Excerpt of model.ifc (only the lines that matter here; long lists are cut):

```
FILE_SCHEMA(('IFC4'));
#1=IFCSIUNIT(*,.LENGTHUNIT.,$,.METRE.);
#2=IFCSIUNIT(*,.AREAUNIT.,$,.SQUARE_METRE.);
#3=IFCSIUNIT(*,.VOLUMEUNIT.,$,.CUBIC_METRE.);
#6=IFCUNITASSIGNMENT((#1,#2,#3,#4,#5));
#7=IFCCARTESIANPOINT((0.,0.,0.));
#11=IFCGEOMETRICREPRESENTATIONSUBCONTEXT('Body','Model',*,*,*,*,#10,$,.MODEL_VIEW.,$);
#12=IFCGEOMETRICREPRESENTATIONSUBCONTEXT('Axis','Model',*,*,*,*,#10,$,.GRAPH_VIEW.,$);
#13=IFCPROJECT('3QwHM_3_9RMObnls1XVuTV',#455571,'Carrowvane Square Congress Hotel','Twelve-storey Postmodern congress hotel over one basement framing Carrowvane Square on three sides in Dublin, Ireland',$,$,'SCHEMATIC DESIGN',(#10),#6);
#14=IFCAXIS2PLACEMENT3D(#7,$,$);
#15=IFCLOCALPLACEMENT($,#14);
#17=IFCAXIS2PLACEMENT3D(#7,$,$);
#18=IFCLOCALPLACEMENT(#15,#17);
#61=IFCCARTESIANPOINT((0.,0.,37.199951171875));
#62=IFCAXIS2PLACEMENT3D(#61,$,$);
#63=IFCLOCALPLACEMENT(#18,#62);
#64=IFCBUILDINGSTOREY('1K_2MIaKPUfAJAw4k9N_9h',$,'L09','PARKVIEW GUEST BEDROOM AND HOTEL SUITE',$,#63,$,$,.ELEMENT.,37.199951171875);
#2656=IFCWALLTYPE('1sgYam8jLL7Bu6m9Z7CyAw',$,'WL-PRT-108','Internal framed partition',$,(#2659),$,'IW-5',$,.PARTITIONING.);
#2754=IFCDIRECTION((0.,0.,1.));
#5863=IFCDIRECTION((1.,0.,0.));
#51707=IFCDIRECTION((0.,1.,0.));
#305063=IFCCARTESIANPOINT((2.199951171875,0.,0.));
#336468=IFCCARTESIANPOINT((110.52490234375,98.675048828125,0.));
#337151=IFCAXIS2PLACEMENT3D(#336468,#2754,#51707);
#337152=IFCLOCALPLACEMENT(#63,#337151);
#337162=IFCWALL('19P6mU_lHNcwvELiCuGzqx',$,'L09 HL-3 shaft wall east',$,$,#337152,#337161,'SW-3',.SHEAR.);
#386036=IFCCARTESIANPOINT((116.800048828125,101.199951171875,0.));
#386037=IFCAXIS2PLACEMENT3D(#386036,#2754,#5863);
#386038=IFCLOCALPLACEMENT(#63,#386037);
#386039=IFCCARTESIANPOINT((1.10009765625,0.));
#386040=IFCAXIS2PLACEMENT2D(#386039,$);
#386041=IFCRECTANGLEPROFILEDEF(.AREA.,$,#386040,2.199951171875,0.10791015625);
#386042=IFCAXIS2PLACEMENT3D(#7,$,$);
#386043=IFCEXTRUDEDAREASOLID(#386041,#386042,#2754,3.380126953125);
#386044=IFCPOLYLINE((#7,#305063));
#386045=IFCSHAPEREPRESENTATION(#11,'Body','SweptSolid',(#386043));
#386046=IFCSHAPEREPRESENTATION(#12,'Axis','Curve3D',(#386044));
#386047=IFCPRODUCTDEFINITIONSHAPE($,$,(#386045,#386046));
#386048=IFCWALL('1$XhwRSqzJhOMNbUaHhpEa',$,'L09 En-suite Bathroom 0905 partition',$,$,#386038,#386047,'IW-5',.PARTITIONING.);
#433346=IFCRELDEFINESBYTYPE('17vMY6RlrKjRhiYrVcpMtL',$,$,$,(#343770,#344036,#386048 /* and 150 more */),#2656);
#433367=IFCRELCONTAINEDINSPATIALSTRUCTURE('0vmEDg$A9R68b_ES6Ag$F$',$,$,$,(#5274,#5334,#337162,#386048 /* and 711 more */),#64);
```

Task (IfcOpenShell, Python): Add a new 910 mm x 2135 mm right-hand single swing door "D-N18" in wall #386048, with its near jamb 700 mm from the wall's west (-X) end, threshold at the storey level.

```python
import numpy as np
import ifcopenshell
import ifcopenshell.api.feature
import ifcopenshell.api.geometry
import ifcopenshell.api.root
import ifcopenshell.api.spatial
import ifcopenshell.geom
import ifcopenshell.util.element
import ifcopenshell.util.placement
import ifcopenshell.util.representation
import ifcopenshell.util.shape
import ifcopenshell.util.unit

model = ifcopenshell.open("model.ifc")
unit_scale = ifcopenshell.util.unit.calculate_unit_scale(model)
settings = ifcopenshell.geom.settings()


def volume(element):
    """Net volume in cubic metres, openings subtracted."""
    shape = ifcopenshell.geom.create_shape(settings, element)
    return ifcopenshell.util.shape.get_volume(shape.geometry)


wall = model.by_guid("1$XhwRSqzJhOMNbUaHhpEa")
storey = ifcopenshell.util.element.get_container(wall, ifc_class="IfcBuildingStorey")
context = ifcopenshell.util.representation.get_context(model, "Model", "Body", "MODEL_VIEW")
before = volume(wall)

width, height, from_end, sill = 0.91, 2.135, 0.7, 0.0  # metres

# The wall runs along its own X axis, and the end named is its -X end.
wall_shape = ifcopenshell.geom.create_shape(settings, wall)
x, y, z = ifcopenshell.util.shape.get_vertices(wall_shape.geometry).T
start = x.min() + from_end
face, thickness = float(y.min()), float(y.max() - y.min())
wall_matrix = ifcopenshell.util.placement.get_local_placement(wall.ObjectPlacement)
level = ifcopenshell.util.placement.get_local_placement(storey.ObjectPlacement)[2, 3]


def in_wall(x, y):
    """Placement at x, y metres in the wall's axes, at sill height."""
    matrix = wall_matrix.copy()
    matrix[:, 3] = wall_matrix @ np.array([x / unit_scale, y / unit_scale, 0.0, 1.0])
    matrix[2, 3] = level + sill / unit_scale
    return matrix


# Opening: a box that overshoots both wall faces by 50 mm.
opening = ifcopenshell.api.root.create_entity(model, ifc_class="IfcOpeningElement", predefined_type="OPENING")
box = ifcopenshell.api.geometry.add_wall_representation(
    model, context=context, length=width, height=height, thickness=thickness + 0.1
)
ifcopenshell.api.geometry.assign_representation(model, product=opening, representation=box)
ifcopenshell.api.geometry.edit_object_placement(model, product=opening, matrix=in_wall(start, face - 0.05), is_si=False)
ifcopenshell.api.feature.add_feature(model, feature=opening, element=wall)

door = ifcopenshell.api.root.create_entity(model, ifc_class="IfcDoor", name="D-N18", predefined_type="DOOR")
door.OverallWidth, door.OverallHeight = width / unit_scale, height / unit_scale
door.OperationType = "SINGLE_SWING_RIGHT"
body = ifcopenshell.api.geometry.add_door_representation(
    model,
    context=context,
    overall_width=door.OverallWidth,
    overall_height=door.OverallHeight,
    operation_type="SINGLE_SWING_RIGHT",
    lining_properties={"LiningDepth": thickness / unit_scale, "ThresholdDepth": thickness / unit_scale},
)
ifcopenshell.api.geometry.assign_representation(model, product=door, representation=body)
ifcopenshell.api.spatial.assign_container(model, products=[door], relating_structure=storey)
ifcopenshell.api.feature.add_filling(model, opening=opening, element=door)

# The lining spans the wall, so the door starts at the wall face.
ifcopenshell.api.geometry.edit_object_placement(model, product=door, matrix=in_wall(start, face), is_si=False)

after = volume(wall)

print(f"wall volume {before:.3f} -> {after:.3f} m3")

model.write("model_updated.ifc")
```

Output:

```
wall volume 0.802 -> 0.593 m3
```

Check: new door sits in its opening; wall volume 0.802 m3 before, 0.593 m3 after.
